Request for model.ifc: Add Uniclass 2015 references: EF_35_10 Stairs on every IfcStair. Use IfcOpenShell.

First a look at what the model holds.

```python
import ifcopenshell

model = ifcopenshell.open("model.ifc")
print(model.schema)
print("classifications:", [c.Name for c in model.by_type("IfcClassification")])
for ifc_class in ("IfcDoor", "IfcRoof", "IfcStair", "IfcWall", "IfcWindow"):
    print(ifc_class, len(model.by_type(ifc_class)))
```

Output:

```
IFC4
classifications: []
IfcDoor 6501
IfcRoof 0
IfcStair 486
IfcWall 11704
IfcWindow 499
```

```python
import ifcopenshell
import ifcopenshell.api.classification

model = ifcopenshell.open("model.ifc")

system = ifcopenshell.api.classification.add_classification(model, classification="Uniclass 2015")

codes = {
    "IfcStair": ("EF_35_10", "Stairs"),
}
for ifc_class, (code, name) in codes.items():
    products = model.by_type(ifc_class)
    ifcopenshell.api.classification.add_reference(
        model, products=products, classification=system, identification=code, name=name
    )
    print(code, len(products))

model.write("model_updated.ifc")
```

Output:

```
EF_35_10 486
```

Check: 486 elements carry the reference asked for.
